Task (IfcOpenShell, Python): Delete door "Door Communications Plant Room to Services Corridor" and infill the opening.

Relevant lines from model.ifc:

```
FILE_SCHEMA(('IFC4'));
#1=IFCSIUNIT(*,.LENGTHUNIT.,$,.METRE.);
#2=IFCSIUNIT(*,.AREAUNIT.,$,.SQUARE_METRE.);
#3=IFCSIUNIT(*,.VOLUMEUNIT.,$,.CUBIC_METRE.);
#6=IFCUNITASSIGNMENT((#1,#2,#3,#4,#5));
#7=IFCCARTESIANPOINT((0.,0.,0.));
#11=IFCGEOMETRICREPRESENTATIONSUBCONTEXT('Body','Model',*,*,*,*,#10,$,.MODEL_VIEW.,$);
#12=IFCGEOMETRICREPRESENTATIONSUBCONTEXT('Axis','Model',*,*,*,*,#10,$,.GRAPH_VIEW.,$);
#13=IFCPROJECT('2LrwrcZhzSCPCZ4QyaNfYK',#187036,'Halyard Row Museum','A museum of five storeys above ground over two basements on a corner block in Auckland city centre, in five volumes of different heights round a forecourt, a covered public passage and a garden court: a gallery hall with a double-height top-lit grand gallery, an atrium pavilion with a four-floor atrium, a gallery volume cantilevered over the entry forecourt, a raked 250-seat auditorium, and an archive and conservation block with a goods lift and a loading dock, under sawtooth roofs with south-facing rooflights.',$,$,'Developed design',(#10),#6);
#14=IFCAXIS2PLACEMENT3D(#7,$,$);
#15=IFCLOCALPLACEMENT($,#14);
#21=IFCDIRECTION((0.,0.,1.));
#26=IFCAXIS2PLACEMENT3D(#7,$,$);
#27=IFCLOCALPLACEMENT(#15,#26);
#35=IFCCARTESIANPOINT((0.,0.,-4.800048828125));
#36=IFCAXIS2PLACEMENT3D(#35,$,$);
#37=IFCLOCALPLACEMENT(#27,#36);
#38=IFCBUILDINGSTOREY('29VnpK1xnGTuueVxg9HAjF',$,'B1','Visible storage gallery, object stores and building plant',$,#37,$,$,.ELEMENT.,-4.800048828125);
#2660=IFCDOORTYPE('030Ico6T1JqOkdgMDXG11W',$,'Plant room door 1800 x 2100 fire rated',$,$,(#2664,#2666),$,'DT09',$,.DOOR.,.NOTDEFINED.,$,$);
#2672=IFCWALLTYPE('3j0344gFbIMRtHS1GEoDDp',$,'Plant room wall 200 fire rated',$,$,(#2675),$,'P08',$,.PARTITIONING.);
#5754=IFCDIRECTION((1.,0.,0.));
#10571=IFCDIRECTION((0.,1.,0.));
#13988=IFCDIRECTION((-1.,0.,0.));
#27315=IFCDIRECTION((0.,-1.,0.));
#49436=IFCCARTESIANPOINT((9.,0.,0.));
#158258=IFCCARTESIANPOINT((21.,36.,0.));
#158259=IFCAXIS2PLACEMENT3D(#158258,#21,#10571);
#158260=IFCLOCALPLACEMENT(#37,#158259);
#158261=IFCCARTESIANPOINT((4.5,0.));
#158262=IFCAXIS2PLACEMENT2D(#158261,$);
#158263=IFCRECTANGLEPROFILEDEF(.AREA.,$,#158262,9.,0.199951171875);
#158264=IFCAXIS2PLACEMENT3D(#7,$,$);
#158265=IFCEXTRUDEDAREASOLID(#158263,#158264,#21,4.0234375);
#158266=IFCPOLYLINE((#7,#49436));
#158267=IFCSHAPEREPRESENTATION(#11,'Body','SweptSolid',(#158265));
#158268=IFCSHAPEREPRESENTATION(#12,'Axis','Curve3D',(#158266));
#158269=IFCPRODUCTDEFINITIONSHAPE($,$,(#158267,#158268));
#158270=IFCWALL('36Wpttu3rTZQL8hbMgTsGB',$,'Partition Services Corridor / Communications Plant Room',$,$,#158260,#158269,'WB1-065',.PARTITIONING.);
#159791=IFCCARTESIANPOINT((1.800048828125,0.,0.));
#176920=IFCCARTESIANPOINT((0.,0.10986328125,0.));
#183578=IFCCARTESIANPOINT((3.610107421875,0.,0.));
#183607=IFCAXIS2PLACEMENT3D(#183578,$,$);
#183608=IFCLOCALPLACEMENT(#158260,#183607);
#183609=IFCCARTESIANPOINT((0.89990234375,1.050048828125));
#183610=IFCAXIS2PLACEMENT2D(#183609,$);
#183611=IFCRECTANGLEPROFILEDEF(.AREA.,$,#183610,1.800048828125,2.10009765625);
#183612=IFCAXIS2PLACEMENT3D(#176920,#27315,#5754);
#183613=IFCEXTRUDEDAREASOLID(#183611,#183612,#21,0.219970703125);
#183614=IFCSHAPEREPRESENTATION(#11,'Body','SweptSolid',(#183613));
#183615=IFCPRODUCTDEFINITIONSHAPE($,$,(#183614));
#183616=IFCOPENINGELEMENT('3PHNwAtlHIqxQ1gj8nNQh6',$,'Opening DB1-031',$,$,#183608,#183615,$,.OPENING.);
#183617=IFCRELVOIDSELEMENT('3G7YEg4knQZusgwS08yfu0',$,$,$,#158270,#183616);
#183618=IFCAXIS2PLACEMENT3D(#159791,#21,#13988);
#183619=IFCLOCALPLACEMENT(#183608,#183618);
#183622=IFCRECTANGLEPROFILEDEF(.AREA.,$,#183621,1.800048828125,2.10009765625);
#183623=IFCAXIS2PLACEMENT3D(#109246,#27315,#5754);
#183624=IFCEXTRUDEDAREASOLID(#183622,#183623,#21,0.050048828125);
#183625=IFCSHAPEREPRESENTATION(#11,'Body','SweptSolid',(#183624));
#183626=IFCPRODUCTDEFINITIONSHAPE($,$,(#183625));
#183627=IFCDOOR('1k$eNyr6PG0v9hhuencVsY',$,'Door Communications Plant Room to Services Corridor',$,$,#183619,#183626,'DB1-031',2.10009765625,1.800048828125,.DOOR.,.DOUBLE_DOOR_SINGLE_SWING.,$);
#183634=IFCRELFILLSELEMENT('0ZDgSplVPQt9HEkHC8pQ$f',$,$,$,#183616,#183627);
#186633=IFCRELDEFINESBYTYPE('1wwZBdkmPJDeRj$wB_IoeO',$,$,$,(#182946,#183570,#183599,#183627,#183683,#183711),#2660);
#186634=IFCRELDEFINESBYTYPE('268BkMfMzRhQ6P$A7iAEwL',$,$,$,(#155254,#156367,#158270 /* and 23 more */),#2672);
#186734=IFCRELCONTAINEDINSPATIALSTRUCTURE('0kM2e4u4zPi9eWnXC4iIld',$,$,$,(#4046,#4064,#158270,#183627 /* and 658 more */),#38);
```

```python
import ifcopenshell
import ifcopenshell.api.feature
import ifcopenshell.api.root
import ifcopenshell.geom
import ifcopenshell.util.shape

model = ifcopenshell.open("model.ifc")
settings = ifcopenshell.geom.settings()


def volume(element):
    """Net volume in cubic metres, openings subtracted."""
    shape = ifcopenshell.geom.create_shape(settings, element)
    return ifcopenshell.util.shape.get_volume(shape.geometry)


door = model.by_guid("1k$eNyr6PG0v9hhuencVsY")
opening = door.FillsVoids[0].RelatingOpeningElement
wall = opening.VoidsElements[0].RelatingBuildingElement
before = volume(wall)

ifcopenshell.api.root.remove_product(model, product=door)
ifcopenshell.api.feature.remove_feature(model, feature=opening)

after = volume(wall)

print(f"wall volume {before:.3f} -> {after:.3f} m3")

model.write("model_v2.ifc")
```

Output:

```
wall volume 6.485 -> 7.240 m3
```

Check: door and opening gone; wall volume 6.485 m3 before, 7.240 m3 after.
